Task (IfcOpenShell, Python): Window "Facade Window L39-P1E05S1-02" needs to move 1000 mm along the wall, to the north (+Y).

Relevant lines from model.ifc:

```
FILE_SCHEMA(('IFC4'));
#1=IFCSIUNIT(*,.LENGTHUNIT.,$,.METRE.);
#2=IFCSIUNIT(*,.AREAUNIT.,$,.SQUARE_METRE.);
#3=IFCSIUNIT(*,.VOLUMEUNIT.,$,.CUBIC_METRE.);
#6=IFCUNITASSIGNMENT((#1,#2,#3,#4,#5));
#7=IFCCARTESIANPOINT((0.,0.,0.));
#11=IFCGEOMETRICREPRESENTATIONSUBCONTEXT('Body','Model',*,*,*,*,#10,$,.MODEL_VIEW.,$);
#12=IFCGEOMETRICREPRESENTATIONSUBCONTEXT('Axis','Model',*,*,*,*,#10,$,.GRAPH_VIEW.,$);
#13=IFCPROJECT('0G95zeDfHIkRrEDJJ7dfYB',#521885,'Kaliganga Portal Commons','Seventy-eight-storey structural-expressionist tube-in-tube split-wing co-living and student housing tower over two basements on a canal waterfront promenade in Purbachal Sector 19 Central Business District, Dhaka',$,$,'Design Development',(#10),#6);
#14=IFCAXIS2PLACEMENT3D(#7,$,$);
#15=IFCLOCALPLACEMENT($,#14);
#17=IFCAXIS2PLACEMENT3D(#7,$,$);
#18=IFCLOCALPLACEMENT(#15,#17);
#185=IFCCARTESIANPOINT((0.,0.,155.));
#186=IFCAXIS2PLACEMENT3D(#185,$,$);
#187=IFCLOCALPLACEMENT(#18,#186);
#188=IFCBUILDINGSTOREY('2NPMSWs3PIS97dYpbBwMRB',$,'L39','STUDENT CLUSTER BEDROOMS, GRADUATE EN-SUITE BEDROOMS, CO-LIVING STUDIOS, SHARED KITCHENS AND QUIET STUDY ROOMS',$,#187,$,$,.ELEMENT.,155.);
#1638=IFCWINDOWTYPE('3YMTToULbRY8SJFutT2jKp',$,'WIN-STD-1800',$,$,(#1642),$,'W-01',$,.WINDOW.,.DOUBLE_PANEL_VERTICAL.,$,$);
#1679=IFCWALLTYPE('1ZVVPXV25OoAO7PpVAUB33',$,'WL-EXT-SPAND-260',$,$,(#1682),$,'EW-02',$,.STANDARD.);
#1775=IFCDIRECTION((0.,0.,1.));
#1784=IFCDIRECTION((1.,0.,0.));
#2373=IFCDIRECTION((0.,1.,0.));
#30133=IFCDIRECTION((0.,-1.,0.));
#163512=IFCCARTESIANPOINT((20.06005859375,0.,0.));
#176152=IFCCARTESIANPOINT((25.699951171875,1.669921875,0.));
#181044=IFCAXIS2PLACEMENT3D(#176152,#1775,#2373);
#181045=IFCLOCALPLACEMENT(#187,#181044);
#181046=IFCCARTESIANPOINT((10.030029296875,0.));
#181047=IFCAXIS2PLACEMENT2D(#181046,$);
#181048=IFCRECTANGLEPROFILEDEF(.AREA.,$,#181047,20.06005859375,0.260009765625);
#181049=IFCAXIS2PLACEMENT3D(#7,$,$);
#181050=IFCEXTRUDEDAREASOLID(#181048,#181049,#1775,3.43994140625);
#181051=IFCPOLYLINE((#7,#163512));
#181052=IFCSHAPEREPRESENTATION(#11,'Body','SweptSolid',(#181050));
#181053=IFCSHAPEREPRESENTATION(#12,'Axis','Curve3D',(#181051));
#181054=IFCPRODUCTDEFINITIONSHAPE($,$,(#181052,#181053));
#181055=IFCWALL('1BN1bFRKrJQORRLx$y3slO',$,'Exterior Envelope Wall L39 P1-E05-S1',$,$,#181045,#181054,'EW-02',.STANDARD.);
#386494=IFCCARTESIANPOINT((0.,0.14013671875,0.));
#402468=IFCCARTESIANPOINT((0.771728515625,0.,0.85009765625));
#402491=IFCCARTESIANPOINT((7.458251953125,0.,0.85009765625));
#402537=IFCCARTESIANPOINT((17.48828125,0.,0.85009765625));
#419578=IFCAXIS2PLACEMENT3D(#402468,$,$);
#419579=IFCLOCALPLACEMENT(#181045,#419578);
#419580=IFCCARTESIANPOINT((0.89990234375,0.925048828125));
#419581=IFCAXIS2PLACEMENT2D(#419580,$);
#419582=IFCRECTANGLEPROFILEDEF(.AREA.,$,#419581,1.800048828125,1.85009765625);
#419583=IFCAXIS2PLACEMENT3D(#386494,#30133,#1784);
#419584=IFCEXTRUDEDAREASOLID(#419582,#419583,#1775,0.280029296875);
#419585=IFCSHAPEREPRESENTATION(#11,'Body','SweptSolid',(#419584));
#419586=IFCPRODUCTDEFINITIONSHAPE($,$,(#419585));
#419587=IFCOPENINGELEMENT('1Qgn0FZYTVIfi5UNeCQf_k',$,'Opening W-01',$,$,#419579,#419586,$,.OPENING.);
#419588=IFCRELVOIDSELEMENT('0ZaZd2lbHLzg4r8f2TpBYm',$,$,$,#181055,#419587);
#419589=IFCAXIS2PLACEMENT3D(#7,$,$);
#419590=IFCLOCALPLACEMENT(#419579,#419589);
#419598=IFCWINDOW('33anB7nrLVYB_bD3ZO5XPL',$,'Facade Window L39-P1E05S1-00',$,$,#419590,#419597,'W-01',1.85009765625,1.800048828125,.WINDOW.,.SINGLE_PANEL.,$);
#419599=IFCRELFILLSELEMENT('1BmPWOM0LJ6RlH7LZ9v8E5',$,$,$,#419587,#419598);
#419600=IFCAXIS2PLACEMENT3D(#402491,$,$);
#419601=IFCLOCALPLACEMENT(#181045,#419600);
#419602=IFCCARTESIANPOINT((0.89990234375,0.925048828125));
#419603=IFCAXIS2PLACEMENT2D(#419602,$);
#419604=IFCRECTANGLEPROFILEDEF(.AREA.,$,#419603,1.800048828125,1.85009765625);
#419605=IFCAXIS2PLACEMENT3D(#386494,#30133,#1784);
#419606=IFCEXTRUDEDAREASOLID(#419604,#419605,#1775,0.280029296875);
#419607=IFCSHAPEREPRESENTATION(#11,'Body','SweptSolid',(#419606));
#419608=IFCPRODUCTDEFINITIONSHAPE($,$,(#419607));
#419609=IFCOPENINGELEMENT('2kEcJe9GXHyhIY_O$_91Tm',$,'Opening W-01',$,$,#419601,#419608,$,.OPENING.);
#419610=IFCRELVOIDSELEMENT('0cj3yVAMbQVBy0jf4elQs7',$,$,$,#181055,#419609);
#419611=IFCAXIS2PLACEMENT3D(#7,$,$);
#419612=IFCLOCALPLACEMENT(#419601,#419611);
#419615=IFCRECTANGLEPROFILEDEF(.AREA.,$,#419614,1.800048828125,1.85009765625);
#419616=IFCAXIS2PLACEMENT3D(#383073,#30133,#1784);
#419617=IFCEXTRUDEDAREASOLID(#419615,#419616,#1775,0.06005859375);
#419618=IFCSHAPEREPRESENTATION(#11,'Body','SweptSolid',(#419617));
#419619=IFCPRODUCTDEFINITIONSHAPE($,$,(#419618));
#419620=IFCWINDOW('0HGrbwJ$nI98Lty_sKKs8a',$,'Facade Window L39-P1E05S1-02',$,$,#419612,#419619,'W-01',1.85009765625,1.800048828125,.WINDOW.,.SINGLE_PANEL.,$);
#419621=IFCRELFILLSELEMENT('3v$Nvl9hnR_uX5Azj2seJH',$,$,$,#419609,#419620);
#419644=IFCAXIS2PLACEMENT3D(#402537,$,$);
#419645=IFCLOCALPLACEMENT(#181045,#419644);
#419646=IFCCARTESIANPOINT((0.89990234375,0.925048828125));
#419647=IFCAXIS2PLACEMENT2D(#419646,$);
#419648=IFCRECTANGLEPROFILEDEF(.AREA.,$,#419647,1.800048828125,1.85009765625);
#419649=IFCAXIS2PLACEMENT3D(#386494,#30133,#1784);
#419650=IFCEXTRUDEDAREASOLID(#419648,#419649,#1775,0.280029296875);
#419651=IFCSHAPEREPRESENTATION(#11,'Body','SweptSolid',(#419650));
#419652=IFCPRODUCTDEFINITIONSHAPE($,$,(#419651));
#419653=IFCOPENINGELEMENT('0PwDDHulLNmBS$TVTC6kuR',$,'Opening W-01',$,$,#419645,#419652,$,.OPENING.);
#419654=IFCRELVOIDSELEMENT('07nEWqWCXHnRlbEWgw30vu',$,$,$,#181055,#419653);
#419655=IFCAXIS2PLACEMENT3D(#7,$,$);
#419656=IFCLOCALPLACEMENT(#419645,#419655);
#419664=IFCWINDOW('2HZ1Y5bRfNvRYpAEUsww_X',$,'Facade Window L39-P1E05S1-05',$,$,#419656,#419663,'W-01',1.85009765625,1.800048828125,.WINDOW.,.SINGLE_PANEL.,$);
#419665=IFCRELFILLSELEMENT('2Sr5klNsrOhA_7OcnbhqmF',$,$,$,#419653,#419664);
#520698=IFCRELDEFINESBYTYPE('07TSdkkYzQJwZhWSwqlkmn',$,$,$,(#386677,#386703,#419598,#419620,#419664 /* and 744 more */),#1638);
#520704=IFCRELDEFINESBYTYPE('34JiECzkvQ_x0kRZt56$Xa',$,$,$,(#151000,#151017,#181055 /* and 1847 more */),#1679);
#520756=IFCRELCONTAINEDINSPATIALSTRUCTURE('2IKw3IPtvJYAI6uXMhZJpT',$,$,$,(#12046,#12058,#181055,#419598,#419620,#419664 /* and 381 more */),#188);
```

```python
import ifcopenshell
import ifcopenshell.api.geometry
import ifcopenshell.util.placement

model = ifcopenshell.open("model.ifc")

window = model.by_id(419620)
opening = window.FillsVoids[0].RelatingOpeningElement
wall = opening.VoidsElements[0].RelatingBuildingElement

wall_matrix = ifcopenshell.util.placement.get_local_placement(wall.ObjectPlacement)
shift = wall_matrix[:3, 0] * 1.0
before = ifcopenshell.util.placement.get_local_placement(window.ObjectPlacement)[:3, 3].copy()

# The window is placed relative to its opening, so it follows when the opening moves.
matrix = ifcopenshell.util.placement.get_local_placement(opening.ObjectPlacement)
matrix[:3, 3] += shift
ifcopenshell.api.geometry.edit_object_placement(
    model, product=opening, matrix=matrix, is_si=False, should_transform_children=True
)

after = ifcopenshell.util.placement.get_local_placement(window.ObjectPlacement)[:3, 3]
print("window moved by", (after - before).round(3) + 0.0)

model.write("model_rev.ifc")
```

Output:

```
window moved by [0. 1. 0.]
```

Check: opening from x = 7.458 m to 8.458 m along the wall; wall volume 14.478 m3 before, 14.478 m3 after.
